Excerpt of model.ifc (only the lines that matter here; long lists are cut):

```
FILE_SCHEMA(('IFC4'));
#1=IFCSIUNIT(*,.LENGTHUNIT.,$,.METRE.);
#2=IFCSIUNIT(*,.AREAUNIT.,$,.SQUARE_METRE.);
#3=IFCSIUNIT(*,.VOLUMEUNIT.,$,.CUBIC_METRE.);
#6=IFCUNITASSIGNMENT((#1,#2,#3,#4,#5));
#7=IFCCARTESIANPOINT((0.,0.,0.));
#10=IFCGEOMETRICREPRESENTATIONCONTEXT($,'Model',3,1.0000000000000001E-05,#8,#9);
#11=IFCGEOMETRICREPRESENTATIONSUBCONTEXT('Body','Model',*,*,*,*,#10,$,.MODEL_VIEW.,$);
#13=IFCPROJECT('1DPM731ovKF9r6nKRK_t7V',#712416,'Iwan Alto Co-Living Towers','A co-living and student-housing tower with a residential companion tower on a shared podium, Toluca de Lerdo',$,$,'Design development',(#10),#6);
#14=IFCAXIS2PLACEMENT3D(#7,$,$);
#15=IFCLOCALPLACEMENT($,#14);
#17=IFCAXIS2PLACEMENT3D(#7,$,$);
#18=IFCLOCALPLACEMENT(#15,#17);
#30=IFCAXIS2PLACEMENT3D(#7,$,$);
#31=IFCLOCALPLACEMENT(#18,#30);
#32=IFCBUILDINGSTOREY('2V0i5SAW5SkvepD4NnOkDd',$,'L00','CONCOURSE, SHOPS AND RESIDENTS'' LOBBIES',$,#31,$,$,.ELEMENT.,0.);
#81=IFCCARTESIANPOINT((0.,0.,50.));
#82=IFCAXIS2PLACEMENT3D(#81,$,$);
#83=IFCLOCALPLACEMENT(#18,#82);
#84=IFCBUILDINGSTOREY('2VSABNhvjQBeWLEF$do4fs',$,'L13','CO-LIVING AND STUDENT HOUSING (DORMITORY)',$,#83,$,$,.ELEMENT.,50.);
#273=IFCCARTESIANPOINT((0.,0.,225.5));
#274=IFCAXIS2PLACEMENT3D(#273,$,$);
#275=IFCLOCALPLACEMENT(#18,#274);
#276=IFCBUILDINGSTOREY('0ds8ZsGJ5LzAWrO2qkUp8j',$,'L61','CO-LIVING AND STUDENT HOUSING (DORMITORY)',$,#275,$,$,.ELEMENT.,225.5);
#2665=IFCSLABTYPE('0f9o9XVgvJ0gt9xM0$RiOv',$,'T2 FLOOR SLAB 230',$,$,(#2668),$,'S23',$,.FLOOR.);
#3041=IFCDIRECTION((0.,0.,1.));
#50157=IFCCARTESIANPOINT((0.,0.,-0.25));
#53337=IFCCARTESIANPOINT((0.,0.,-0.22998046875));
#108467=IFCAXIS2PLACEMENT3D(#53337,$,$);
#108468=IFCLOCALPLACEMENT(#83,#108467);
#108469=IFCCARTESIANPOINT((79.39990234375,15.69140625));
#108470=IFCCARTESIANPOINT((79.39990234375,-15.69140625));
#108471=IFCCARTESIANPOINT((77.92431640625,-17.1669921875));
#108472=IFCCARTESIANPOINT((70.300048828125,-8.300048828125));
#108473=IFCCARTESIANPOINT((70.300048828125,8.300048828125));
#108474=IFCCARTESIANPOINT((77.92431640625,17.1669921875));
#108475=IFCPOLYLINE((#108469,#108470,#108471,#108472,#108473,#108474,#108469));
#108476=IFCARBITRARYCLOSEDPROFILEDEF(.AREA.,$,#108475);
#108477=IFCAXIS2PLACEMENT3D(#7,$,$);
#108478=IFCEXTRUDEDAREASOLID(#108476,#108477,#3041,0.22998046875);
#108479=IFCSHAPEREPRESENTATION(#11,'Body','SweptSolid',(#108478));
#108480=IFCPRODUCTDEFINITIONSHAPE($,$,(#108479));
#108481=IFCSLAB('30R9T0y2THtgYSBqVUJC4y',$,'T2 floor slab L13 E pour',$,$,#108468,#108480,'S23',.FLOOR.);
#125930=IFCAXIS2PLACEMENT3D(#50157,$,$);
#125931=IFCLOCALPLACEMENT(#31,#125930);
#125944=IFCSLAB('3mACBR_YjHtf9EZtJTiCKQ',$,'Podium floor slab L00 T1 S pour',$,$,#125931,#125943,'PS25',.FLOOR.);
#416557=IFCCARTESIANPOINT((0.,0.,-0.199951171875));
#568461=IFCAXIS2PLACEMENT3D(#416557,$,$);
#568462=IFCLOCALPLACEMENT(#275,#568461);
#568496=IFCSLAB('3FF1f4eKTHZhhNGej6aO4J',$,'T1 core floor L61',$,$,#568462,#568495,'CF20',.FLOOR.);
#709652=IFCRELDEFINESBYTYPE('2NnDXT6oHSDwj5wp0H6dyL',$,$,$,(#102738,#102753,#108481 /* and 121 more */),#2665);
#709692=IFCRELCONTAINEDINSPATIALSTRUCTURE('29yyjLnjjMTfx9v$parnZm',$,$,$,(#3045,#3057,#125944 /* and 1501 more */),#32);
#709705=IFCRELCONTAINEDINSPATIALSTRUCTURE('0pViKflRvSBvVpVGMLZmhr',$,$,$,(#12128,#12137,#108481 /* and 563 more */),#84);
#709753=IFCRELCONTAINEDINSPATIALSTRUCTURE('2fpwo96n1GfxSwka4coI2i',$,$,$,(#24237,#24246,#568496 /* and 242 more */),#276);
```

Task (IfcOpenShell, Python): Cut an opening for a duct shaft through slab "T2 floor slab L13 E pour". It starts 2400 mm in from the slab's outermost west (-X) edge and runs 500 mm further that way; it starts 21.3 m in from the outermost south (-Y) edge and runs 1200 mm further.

```python
import numpy as np
import ifcopenshell
import ifcopenshell.api.feature
import ifcopenshell.api.geometry
import ifcopenshell.api.root
import ifcopenshell.geom
import ifcopenshell.util.placement
import ifcopenshell.util.representation
import ifcopenshell.util.shape
import ifcopenshell.util.unit

model = ifcopenshell.open("model.ifc")
unit_scale = ifcopenshell.util.unit.calculate_unit_scale(model)
settings = ifcopenshell.geom.settings()


def volume(element):
    """Net volume in cubic metres, openings subtracted."""
    shape = ifcopenshell.geom.create_shape(settings, element)
    return ifcopenshell.util.shape.get_volume(shape.geometry)


slab = model.by_id(108481)
before = volume(slab)

# Extent in the slab's own axes, in metres. The edges named are its -X and -Y sides.
slab_shape = ifcopenshell.geom.create_shape(settings, slab)
vertices = ifcopenshell.util.shape.get_vertices(slab_shape.geometry)
x_min, y_min, bottom = vertices.min(axis=0)
top = vertices[:, 2].max()

opening = ifcopenshell.api.root.create_entity(model, ifc_class="IfcOpeningElement", name="Duct shaft opening", predefined_type="OPENING")
context = ifcopenshell.util.representation.get_context(model, "Model", "Body", "MODEL_VIEW")
width, depth = 0.5, 1.2
outline = [(0.0, 0.0), (width, 0.0), (width, depth), (0.0, depth), (0.0, 0.0)]
# Overshoot both faces by 50 mm so the cut is clean.
shape = ifcopenshell.api.geometry.add_slab_representation(
    model, context=context, depth=top - bottom + 0.1, polyline=outline
)
ifcopenshell.api.geometry.assign_representation(model, product=opening, representation=shape)

matrix = ifcopenshell.util.placement.get_local_placement(slab.ObjectPlacement)
matrix[:, 3] = matrix @ np.append(np.array([x_min + 2.4, y_min + 21.3, bottom - 0.05]) / unit_scale, 1.0)
ifcopenshell.api.geometry.edit_object_placement(model, product=opening, matrix=matrix, is_si=False)
ifcopenshell.api.feature.add_feature(model, feature=opening, element=slab)

after = volume(slab)

print(f"slab volume {before:.3f} -> {after:.3f} m3")

model.write("model_updated.ifc")
```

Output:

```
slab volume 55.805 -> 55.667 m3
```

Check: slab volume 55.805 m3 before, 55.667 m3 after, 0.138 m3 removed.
